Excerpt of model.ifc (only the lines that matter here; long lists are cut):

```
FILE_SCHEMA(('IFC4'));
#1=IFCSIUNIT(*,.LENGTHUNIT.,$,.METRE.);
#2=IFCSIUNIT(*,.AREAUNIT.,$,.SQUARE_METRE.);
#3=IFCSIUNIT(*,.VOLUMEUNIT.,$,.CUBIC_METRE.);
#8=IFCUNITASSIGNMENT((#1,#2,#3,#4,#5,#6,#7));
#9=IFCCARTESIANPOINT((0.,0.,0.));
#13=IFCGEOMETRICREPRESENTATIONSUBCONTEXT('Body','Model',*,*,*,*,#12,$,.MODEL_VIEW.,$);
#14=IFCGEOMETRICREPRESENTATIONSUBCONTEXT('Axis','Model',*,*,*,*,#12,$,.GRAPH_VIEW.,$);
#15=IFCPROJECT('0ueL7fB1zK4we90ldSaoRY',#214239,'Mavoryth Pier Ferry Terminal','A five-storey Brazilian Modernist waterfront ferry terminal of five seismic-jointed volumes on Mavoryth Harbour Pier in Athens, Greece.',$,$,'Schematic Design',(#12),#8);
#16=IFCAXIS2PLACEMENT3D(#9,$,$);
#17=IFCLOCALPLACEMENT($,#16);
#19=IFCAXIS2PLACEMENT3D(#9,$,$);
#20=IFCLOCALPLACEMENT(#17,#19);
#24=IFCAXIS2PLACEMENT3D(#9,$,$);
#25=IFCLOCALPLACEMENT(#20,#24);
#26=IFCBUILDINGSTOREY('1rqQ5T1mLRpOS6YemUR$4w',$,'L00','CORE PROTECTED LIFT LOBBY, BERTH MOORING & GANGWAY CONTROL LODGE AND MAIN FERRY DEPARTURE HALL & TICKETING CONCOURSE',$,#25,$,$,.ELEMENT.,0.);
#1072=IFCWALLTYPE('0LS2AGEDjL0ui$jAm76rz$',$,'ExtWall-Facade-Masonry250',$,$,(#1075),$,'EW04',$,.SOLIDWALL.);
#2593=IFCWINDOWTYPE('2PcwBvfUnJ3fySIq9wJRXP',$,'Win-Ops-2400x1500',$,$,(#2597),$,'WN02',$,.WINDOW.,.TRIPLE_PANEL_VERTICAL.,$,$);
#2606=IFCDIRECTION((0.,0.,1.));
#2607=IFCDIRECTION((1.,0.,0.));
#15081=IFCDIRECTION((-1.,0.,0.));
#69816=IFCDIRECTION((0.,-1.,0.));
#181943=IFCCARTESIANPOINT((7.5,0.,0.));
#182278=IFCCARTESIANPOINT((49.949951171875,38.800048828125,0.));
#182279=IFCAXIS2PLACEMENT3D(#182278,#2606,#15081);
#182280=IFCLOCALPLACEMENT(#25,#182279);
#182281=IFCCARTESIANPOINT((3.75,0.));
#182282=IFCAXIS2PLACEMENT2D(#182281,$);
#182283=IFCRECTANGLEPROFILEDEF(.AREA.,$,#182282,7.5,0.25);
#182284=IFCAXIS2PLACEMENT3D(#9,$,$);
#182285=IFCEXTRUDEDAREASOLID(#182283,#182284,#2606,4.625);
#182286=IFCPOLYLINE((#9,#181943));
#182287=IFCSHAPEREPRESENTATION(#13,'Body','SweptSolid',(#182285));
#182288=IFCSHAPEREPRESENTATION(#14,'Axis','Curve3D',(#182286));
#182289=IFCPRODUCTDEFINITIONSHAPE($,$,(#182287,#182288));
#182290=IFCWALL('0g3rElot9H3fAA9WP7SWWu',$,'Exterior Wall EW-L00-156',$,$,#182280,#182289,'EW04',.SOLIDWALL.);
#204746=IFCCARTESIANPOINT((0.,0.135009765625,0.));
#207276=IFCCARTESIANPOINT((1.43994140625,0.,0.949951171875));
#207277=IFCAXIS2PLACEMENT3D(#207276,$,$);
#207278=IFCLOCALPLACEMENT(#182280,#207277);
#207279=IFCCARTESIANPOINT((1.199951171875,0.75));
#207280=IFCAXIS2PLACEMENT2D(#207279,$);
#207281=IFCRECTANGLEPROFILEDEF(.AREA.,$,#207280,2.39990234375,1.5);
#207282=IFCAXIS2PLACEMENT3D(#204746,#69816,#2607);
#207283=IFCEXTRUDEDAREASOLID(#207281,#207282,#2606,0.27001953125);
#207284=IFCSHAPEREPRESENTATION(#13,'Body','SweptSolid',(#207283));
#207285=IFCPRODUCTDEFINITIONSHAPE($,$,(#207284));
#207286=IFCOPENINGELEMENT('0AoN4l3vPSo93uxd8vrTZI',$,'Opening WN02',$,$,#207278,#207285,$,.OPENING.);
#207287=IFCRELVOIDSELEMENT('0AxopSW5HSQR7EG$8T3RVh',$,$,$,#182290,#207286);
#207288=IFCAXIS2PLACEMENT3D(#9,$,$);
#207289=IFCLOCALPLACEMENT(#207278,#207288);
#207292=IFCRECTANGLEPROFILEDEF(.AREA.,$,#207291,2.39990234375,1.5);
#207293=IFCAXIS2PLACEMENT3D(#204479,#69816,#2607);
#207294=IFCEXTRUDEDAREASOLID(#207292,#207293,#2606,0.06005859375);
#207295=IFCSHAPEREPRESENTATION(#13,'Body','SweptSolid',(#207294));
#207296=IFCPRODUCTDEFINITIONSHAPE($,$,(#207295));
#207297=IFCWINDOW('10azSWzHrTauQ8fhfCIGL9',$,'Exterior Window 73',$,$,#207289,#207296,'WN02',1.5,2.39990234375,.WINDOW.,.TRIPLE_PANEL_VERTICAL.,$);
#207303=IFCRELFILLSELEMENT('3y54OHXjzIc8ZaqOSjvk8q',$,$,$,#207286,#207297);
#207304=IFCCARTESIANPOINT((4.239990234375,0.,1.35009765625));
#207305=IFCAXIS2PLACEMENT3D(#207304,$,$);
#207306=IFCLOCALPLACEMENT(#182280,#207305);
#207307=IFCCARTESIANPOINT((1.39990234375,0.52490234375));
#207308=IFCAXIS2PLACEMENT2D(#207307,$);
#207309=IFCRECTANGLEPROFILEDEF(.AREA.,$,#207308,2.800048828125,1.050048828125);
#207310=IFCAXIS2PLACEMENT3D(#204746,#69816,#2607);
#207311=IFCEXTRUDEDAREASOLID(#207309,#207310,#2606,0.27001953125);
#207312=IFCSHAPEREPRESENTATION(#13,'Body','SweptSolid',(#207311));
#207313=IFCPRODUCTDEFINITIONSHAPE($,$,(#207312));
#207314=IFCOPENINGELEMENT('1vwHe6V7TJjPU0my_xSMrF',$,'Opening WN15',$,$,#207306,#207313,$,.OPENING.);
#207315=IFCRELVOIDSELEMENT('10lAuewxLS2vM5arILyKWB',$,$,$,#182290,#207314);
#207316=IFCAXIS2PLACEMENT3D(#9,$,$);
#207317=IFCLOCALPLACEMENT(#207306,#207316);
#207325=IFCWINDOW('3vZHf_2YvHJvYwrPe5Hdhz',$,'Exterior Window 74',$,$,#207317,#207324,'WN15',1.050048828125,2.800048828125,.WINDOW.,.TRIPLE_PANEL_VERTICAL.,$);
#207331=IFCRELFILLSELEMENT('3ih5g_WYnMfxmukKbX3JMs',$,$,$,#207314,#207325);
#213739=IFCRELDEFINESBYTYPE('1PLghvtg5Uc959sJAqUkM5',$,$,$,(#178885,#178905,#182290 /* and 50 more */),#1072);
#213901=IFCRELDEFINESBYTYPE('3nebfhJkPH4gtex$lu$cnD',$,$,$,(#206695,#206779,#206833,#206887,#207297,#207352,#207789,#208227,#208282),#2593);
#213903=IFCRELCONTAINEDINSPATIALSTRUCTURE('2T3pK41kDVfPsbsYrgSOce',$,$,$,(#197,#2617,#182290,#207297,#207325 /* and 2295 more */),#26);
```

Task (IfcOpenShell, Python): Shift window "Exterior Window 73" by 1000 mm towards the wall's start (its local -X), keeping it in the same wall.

```python
import ifcopenshell
import ifcopenshell.api.geometry
import ifcopenshell.util.placement
import ifcopenshell.util.unit

model = ifcopenshell.open("model.ifc")
unit_scale = ifcopenshell.util.unit.calculate_unit_scale(model)

window = model.by_guid("10azSWzHrTauQ8fhfCIGL9")
opening = window.FillsVoids[0].RelatingOpeningElement
wall = opening.VoidsElements[0].RelatingBuildingElement

wall_matrix = ifcopenshell.util.placement.get_local_placement(wall.ObjectPlacement)
shift = wall_matrix[:3, 0] * -1 / unit_scale
before = ifcopenshell.util.placement.get_local_placement(window.ObjectPlacement)[:3, 3].copy()

# The window is placed relative to its opening, so it follows when the opening moves.
matrix = ifcopenshell.util.placement.get_local_placement(opening.ObjectPlacement)
matrix[:3, 3] += shift
ifcopenshell.api.geometry.edit_object_placement(
    model, product=opening, matrix=matrix, is_si=False, should_transform_children=True
)

after = ifcopenshell.util.placement.get_local_placement(window.ObjectPlacement)[:3, 3]
print("window moved by", (after - before).round(3) + 0.0)

model.write("model_updated.ifc")
```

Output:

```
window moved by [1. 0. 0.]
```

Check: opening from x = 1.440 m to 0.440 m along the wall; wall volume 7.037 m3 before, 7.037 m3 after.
